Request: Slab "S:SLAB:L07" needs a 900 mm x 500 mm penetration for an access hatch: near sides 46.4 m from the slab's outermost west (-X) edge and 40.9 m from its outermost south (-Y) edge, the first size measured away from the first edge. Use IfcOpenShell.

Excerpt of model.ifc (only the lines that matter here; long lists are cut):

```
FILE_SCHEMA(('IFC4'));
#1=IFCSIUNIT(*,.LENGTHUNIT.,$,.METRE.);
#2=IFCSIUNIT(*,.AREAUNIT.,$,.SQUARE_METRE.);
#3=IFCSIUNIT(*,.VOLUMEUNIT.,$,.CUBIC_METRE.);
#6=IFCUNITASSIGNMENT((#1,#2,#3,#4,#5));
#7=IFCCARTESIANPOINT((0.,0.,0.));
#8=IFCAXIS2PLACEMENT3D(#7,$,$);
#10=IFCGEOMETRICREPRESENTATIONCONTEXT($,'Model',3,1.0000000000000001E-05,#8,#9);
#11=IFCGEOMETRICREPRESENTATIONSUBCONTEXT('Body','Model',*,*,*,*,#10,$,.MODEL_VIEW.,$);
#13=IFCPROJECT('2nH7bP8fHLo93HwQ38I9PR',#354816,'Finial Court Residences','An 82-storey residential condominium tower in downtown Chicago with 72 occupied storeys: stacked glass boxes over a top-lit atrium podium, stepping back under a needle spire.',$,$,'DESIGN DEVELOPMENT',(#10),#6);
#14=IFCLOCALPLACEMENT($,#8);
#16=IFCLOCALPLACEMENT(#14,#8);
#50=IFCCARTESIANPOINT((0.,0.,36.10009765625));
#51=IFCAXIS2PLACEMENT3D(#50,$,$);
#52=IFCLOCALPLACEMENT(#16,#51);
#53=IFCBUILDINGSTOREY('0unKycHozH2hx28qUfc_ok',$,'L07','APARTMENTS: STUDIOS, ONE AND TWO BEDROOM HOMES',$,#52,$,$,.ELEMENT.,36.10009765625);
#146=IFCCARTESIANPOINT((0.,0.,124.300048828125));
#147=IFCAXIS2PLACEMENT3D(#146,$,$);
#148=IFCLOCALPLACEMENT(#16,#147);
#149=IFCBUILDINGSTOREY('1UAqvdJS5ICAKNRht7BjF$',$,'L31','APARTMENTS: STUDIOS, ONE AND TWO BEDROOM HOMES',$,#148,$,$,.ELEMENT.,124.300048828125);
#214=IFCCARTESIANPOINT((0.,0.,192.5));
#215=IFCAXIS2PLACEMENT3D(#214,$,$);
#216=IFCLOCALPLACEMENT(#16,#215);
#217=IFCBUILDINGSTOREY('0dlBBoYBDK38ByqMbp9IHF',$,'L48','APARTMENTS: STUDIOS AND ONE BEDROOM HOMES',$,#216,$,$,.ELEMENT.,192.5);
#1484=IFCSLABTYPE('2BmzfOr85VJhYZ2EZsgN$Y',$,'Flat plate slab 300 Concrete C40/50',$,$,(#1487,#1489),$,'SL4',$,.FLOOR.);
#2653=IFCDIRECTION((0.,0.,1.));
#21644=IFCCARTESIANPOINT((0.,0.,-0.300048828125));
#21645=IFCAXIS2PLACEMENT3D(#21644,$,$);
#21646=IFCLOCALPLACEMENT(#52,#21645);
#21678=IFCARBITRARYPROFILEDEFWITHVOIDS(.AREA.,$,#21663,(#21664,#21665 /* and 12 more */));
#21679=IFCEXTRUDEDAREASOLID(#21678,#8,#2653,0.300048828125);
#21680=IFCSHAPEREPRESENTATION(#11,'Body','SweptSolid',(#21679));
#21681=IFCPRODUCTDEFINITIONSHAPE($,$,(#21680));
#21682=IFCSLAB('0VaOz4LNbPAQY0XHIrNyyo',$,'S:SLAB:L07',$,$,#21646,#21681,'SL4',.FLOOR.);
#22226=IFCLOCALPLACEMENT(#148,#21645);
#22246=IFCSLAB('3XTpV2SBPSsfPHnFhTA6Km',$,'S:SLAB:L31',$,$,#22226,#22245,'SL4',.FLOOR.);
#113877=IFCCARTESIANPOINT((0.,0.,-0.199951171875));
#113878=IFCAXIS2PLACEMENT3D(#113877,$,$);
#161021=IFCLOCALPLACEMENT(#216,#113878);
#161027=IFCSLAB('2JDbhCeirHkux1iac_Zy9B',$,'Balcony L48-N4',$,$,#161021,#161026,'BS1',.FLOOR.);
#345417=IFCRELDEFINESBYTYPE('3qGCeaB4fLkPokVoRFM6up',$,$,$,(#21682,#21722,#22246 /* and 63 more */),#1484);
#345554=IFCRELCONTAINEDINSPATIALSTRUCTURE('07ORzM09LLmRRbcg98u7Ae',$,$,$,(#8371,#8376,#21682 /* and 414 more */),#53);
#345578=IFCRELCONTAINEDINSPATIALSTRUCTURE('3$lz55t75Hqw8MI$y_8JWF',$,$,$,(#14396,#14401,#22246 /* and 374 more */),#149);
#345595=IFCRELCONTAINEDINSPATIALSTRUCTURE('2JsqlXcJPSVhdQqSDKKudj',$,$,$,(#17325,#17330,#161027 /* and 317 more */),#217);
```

```python
import numpy as np
import ifcopenshell
import ifcopenshell.api.feature
import ifcopenshell.api.geometry
import ifcopenshell.api.root
import ifcopenshell.geom
import ifcopenshell.util.placement
import ifcopenshell.util.representation
import ifcopenshell.util.shape
import ifcopenshell.util.unit

model = ifcopenshell.open("model.ifc")
unit_scale = ifcopenshell.util.unit.calculate_unit_scale(model)
settings = ifcopenshell.geom.settings()


def volume(element):
    """Net volume in cubic metres, openings subtracted."""
    shape = ifcopenshell.geom.create_shape(settings, element)
    return ifcopenshell.util.shape.get_volume(shape.geometry)


slab = model.by_guid("0VaOz4LNbPAQY0XHIrNyyo")
before = volume(slab)

# Extent in the slab's own axes, in metres. The edges named are its -X and -Y sides.
slab_shape = ifcopenshell.geom.create_shape(settings, slab)
vertices = ifcopenshell.util.shape.get_vertices(slab_shape.geometry)
x_min, y_min, bottom = vertices.min(axis=0)
top = vertices[:, 2].max()

opening = ifcopenshell.api.root.create_entity(model, ifc_class="IfcOpeningElement", name="Access hatch opening", predefined_type="OPENING")
context = ifcopenshell.util.representation.get_context(model, "Model", "Body", "MODEL_VIEW")
width, depth = 0.9, 0.5
outline = [(0.0, 0.0), (width, 0.0), (width, depth), (0.0, depth), (0.0, 0.0)]
# Overshoot both faces by 50 mm so the cut is clean.
shape = ifcopenshell.api.geometry.add_slab_representation(
    model, context=context, depth=top - bottom + 0.1, polyline=outline
)
ifcopenshell.api.geometry.assign_representation(model, product=opening, representation=shape)

matrix = ifcopenshell.util.placement.get_local_placement(slab.ObjectPlacement)
matrix[:, 3] = matrix @ np.append(np.array([x_min + 46.4, y_min + 40.9, bottom - 0.05]) / unit_scale, 1.0)
ifcopenshell.api.geometry.edit_object_placement(model, product=opening, matrix=matrix, is_si=False)
ifcopenshell.api.feature.add_feature(model, feature=opening, element=slab)

after = volume(slab)

print(f"slab volume {before:.3f} -> {after:.3f} m3")

model.write("model_rev.ifc")
```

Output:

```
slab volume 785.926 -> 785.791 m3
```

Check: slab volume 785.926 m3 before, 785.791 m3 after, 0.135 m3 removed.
